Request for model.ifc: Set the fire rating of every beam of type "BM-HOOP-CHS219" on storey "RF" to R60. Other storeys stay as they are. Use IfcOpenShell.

First a look at what the model holds.

```python
import ifcopenshell
import ifcopenshell.util.element

model = ifcopenshell.open("model.ifc")
print(model.schema)
storey = next(s for s in model.by_type("IfcBuildingStorey") if s.Name == "RF")
beams = [e for e in ifcopenshell.util.element.get_decomposition(storey) if e.is_a("IfcBeam")]
seen = {}
for e in beams:
    element_type = ifcopenshell.util.element.get_type(e)
    key = (element_type.Name if element_type != e and element_type else None, ifcopenshell.util.element.get_pset(e, "Pset_BeamCommon", "FireRating"))
    seen[key] = seen.get(key, 0) + 1
for (name, value), count in sorted(seen.items(), key=str):
    print(count, "x", name, "|", value)
```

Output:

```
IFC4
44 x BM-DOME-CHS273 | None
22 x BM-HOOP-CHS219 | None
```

```python
import ifcopenshell
import ifcopenshell.api.pset
import ifcopenshell.util.element

model = ifcopenshell.open("model.ifc")

storey = next(s for s in model.by_type("IfcBuildingStorey") if s.Name == "RF")
beams = [e for e in ifcopenshell.util.element.get_decomposition(storey) if e.is_a("IfcBeam")]

count = 0
for e in beams:
    element_type = ifcopenshell.util.element.get_type(e)
    if element_type in (None, e) or element_type.Name != "BM-HOOP-CHS219":
        continue
    # add_pset returns the element's existing set when there is one.
    pset = ifcopenshell.api.pset.add_pset(model, product=e, name="Pset_BeamCommon")
    ifcopenshell.api.pset.edit_pset(model, pset=pset, properties={"FireRating": "R60"})
    count += 1

print(count, "beams updated")

model.write("model_updated.ifc")
```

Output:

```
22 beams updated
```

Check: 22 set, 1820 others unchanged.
